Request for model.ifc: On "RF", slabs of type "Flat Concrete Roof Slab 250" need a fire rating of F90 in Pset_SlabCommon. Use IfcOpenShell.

First a look at what the model holds.

```python
import ifcopenshell
import ifcopenshell.util.element

model = ifcopenshell.open("model.ifc")
print(model.schema)
storey = next(s for s in model.by_type("IfcBuildingStorey") if s.Name == "RF")
slabs = [e for e in ifcopenshell.util.element.get_decomposition(storey) if e.is_a("IfcSlab")]
seen = {}
for e in slabs:
    element_type = ifcopenshell.util.element.get_type(e)
    key = (element_type.Name if element_type != e and element_type else None, ifcopenshell.util.element.get_pset(e, "Pset_SlabCommon", "FireRating"))
    seen[key] = seen.get(key, 0) + 1
for (name, value), count in sorted(seen.items(), key=str):
    print(count, "x", name, "|", value)
```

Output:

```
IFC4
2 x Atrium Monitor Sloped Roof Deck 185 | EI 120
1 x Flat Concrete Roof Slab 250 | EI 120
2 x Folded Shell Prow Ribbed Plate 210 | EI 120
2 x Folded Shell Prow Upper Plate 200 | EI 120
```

```python
import ifcopenshell
import ifcopenshell.api.pset
import ifcopenshell.util.element

model = ifcopenshell.open("model.ifc")

storey = next(s for s in model.by_type("IfcBuildingStorey") if s.Name == "RF")
slabs = [e for e in ifcopenshell.util.element.get_decomposition(storey) if e.is_a("IfcSlab")]

count = 0
for e in slabs:
    element_type = ifcopenshell.util.element.get_type(e)
    if element_type in (None, e) or element_type.Name != "Flat Concrete Roof Slab 250":
        continue
    # add_pset returns the element's existing set when there is one.
    pset = ifcopenshell.api.pset.add_pset(model, product=e, name="Pset_SlabCommon")
    ifcopenshell.api.pset.edit_pset(model, pset=pset, properties={"FireRating": "F90"})
    count += 1

print(count, "slabs updated")

model.write("model_v2.ifc")
```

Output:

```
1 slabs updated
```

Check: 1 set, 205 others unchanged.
